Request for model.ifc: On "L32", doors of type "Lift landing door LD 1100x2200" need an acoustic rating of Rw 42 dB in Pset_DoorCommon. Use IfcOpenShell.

First a look at what the model holds.

```python
import ifcopenshell
import ifcopenshell.util.element

model = ifcopenshell.open("model.ifc")
print(model.schema)
storey = next(s for s in model.by_type("IfcBuildingStorey") if s.Name == "L32")
doors = [e for e in ifcopenshell.util.element.get_decomposition(storey) if e.is_a("IfcDoor")]
seen = {}
for e in doors:
    element_type = ifcopenshell.util.element.get_type(e)
    key = (element_type.Name if element_type != e and element_type else None, ifcopenshell.util.element.get_pset(e, "Pset_DoorCommon", "AcousticRating"))
    seen[key] = seen.get(key, 0) + 1
for (name, value), count in sorted(seen.items(), key=str):
    print(count, "x", name, "|", value)
```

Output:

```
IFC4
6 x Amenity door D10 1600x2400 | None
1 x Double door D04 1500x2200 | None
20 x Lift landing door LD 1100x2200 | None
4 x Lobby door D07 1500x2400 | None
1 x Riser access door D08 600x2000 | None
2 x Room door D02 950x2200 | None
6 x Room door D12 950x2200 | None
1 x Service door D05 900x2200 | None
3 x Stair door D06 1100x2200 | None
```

```python
import ifcopenshell
import ifcopenshell.api.pset
import ifcopenshell.util.element

model = ifcopenshell.open("model.ifc")

storey = next(s for s in model.by_type("IfcBuildingStorey") if s.Name == "L32")
doors = [e for e in ifcopenshell.util.element.get_decomposition(storey) if e.is_a("IfcDoor")]

count = 0
for e in doors:
    element_type = ifcopenshell.util.element.get_type(e)
    if element_type in (None, e) or element_type.Name != "Lift landing door LD 1100x2200":
        continue
    found = ifcopenshell.util.element.get_pset(e, "Pset_DoorCommon", should_inherit=False)
    if found:
        pset = model.by_id(found["id"])
        if len(ifcopenshell.util.element.get_elements_by_pset(pset)) > 1:
            pset = ifcopenshell.api.pset.unshare_pset(model, products=[e], pset=pset)[0]
    else:
        pset = ifcopenshell.api.pset.add_pset(model, product=e, name="Pset_DoorCommon")
    ifcopenshell.api.pset.edit_pset(model, pset=pset, properties={"AcousticRating": "Rw 42 dB"})
    count += 1

print(count, "doors updated")

model.write("model_edited.ifc")
```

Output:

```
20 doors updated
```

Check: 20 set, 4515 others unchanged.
